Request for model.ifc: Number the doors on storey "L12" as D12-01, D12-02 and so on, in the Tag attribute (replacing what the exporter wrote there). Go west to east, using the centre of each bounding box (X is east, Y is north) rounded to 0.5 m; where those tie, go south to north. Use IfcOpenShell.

First a look at what the model holds.

```python
import ifcopenshell
import ifcopenshell.util.element
import ifcopenshell.util.placement

model = ifcopenshell.open("model.ifc")
print(model.schema)
storey = next(s for s in model.by_type("IfcBuildingStorey") if s.Name == "L12")
doors = [e for e in ifcopenshell.util.element.get_decomposition(storey) if e.is_a("IfcDoor")]
for e in sorted(doors, key=lambda e: e.id()):
    origin = ifcopenshell.util.placement.get_local_placement(e.ObjectPlacement)[:3, 3]
    print(e.id(), e.Tag, e.Name, origin.round(2) + 0.0, sep=" | ")
```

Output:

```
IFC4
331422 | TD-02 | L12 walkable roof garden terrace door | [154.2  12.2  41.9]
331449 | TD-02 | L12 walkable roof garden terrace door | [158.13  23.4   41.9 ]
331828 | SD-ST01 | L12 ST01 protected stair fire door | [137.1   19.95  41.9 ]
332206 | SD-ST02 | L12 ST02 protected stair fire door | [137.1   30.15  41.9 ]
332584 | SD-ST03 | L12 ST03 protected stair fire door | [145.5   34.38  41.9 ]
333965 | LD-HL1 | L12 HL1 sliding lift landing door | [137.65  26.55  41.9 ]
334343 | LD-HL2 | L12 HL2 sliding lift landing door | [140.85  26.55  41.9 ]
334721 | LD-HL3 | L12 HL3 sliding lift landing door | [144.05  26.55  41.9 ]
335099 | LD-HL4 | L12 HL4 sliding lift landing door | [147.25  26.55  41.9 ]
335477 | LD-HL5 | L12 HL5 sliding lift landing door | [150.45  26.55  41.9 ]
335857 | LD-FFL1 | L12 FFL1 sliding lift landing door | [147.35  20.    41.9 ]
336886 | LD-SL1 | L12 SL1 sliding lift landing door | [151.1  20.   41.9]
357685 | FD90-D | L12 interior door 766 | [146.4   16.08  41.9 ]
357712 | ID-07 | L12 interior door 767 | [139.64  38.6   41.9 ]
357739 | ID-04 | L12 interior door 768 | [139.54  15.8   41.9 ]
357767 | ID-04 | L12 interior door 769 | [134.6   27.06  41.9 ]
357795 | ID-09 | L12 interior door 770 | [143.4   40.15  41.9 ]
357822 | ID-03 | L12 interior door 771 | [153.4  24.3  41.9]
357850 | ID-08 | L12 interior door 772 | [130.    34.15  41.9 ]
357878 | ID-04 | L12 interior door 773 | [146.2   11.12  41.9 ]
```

```python
import ifcopenshell
import ifcopenshell.geom
import ifcopenshell.util.element
import ifcopenshell.util.shape

model = ifcopenshell.open("model.ifc")
settings = ifcopenshell.geom.settings()
settings.set("use-world-coords", True)


def centre(element):
    shape = ifcopenshell.geom.create_shape(settings, element)
    return ifcopenshell.util.shape.get_bbox_centroid(shape.geometry)


storey = next(s for s in model.by_type("IfcBuildingStorey") if s.Name == "L12")
doors = [e for e in ifcopenshell.util.element.get_decomposition(storey) if e.is_a("IfcDoor")]

# Insertion points can sit at a corner or the storey origin, so sort by the geometry (in metres).
centres = {e: centre(e) for e in doors}
doors.sort(key=lambda e: (round(centres[e][0] / 0.5), centres[e][1]))

for i, e in enumerate(doors, start=1):
    number = f"D12-{i:02d}"
    e.Tag = number
    print(e.id(), number)

model.write("model_updated.ifc")
```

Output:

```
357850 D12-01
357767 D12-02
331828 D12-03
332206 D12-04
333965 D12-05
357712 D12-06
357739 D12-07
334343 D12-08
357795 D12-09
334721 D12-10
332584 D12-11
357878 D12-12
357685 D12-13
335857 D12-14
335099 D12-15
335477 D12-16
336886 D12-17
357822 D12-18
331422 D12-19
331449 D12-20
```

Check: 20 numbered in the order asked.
